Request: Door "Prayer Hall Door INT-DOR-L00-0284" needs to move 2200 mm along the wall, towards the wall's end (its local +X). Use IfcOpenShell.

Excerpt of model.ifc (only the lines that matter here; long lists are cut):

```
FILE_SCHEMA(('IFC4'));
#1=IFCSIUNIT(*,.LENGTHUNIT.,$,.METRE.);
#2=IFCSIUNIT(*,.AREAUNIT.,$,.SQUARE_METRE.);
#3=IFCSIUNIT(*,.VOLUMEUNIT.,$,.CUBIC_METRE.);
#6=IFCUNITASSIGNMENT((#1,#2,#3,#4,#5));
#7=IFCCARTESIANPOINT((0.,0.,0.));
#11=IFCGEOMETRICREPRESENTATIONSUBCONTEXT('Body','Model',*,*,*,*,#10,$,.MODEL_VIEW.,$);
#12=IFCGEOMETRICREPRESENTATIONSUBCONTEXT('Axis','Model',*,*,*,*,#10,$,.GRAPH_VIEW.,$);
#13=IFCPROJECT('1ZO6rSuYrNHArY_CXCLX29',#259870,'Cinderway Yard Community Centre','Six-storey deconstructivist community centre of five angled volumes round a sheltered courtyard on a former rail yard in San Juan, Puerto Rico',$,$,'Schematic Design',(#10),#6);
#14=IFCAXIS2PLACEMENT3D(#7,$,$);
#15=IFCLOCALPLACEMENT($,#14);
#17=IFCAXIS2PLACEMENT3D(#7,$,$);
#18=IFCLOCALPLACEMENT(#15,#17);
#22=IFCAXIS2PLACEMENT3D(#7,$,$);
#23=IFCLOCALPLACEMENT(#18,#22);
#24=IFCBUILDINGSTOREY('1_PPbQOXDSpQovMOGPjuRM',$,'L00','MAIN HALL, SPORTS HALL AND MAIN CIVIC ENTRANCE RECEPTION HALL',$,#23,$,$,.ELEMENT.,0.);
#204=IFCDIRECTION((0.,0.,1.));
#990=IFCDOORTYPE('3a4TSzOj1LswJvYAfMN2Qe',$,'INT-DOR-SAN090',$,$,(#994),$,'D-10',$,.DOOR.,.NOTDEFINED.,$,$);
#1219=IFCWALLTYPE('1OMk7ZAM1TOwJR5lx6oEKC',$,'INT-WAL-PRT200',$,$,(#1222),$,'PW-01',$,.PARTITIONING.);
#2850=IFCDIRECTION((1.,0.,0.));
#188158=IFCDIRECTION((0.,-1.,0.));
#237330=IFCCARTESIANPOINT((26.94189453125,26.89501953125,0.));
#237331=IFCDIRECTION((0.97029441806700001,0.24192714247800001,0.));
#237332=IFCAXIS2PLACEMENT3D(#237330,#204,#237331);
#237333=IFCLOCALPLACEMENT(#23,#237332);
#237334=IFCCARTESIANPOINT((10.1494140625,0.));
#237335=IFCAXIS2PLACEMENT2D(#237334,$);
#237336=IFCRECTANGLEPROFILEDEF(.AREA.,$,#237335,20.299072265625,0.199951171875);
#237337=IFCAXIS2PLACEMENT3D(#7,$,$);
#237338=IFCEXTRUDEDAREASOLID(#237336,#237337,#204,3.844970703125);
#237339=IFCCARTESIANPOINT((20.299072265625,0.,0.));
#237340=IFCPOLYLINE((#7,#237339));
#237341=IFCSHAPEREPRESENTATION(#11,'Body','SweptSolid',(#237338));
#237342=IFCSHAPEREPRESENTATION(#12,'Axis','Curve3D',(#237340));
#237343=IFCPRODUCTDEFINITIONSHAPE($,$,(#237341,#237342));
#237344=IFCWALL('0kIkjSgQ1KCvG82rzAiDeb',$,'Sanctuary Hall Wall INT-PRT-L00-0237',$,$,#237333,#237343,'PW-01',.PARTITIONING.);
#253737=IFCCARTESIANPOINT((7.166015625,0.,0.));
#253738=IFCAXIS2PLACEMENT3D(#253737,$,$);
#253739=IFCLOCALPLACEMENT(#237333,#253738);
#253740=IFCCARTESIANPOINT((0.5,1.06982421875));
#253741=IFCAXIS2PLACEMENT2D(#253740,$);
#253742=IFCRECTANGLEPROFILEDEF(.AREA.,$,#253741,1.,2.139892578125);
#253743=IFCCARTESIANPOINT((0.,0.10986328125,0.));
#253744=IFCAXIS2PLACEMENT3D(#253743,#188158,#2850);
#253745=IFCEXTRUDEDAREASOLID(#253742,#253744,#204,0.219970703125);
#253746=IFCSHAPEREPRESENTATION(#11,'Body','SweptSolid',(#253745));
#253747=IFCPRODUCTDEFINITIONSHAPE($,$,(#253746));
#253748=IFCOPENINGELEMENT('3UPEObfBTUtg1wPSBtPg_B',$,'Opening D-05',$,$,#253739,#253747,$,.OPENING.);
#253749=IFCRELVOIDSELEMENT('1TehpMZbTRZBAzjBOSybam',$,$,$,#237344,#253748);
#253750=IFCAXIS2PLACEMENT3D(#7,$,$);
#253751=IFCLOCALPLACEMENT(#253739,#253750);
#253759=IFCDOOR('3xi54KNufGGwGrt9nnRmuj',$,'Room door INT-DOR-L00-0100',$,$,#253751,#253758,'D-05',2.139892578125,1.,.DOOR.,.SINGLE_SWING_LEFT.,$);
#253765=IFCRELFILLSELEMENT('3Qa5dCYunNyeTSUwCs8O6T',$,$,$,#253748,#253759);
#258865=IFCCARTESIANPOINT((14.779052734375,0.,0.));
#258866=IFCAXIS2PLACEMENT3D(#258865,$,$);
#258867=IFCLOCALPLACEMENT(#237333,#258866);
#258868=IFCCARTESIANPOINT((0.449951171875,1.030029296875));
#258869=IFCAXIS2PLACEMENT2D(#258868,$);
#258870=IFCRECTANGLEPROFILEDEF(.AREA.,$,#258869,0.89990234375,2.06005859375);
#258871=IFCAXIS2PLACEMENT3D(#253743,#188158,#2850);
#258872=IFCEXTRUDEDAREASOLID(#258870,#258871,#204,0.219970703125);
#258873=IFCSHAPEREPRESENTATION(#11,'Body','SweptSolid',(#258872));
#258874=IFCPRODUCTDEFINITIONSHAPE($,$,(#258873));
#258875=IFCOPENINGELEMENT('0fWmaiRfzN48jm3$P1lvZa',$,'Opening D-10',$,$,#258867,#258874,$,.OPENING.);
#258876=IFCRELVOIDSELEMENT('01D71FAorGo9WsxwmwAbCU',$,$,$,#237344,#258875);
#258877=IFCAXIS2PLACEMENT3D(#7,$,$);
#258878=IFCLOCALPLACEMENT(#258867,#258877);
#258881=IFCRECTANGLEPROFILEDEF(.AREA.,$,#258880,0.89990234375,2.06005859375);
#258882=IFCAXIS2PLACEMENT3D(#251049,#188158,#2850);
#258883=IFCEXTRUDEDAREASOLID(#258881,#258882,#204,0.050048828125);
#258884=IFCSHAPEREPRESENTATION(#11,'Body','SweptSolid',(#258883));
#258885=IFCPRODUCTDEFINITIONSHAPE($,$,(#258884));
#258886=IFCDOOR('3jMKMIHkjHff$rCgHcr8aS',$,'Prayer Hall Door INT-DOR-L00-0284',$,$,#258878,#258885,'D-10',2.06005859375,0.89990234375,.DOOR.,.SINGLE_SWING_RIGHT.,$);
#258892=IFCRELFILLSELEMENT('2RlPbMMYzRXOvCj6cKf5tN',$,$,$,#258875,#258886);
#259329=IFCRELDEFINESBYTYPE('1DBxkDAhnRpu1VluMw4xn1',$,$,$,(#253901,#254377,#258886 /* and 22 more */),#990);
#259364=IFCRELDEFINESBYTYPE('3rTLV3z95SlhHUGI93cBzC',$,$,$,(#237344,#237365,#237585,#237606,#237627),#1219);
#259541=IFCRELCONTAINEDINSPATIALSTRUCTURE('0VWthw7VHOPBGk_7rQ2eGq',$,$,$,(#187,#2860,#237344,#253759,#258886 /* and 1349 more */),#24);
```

```python
import ifcopenshell
import ifcopenshell.api.geometry
import ifcopenshell.util.placement
import ifcopenshell.util.unit

model = ifcopenshell.open("model.ifc")
unit_scale = ifcopenshell.util.unit.calculate_unit_scale(model)

door = model.by_id(258886)
opening = door.FillsVoids[0].RelatingOpeningElement
wall = opening.VoidsElements[0].RelatingBuildingElement

wall_matrix = ifcopenshell.util.placement.get_local_placement(wall.ObjectPlacement)
shift = wall_matrix[:3, 0] * 2.2 / unit_scale
before = ifcopenshell.util.placement.get_local_placement(door.ObjectPlacement)[:3, 3].copy()

# The door is placed relative to its opening, so it follows when the opening moves.
matrix = ifcopenshell.util.placement.get_local_placement(opening.ObjectPlacement)
matrix[:3, 3] += shift
ifcopenshell.api.geometry.edit_object_placement(
    model, product=opening, matrix=matrix, is_si=False, should_transform_children=True
)

after = ifcopenshell.util.placement.get_local_placement(door.ObjectPlacement)[:3, 3]
print("door moved by", (after - before).round(3) + 0.0)

model.write("model_updated.ifc")
```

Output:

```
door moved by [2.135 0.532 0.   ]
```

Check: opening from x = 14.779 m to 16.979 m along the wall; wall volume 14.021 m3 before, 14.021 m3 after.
